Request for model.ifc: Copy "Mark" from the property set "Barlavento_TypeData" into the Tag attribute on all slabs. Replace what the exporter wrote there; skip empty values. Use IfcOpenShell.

First a look at what the model holds.

```python
import ifcopenshell
import ifcopenshell.util.element

model = ifcopenshell.open("model.ifc")
print(model.schema)
slabs = model.by_type("IfcSlab")
print(len(slabs), "slabs")
for e in slabs[:8]:
    source = ifcopenshell.util.element.get_pset(e, "Barlavento_TypeData", "Mark")
    target = e.Tag
    print(e.id(), repr(source), repr(target), sep=" | ")
```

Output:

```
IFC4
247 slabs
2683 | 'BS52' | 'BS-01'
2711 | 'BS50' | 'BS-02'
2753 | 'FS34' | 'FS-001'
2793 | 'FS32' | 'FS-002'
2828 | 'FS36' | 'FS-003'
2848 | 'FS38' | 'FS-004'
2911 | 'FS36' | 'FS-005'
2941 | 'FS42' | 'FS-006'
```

```python
import ifcopenshell
import ifcopenshell.util.element

model = ifcopenshell.open("model.ifc")

count = 0
for e in model.by_type("IfcSlab"):
    value = ifcopenshell.util.element.get_pset(e, "Barlavento_TypeData", "Mark")
    current = e.Tag
    if not value or not value.strip() or current == value:
        continue
    e.Tag = value
    count += 1

print(count, "slabs updated")

model.write("model_v2.ifc")
```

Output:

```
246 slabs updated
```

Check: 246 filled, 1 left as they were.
